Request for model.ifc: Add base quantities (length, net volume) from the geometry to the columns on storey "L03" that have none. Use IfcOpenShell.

First a look at what the model holds.

```python
import ifcopenshell
import ifcopenshell.util.element
import ifcopenshell.util.unit

model = ifcopenshell.open("model.ifc")
print(model.schema)
for unit_type in ("LENGTHUNIT", "AREAUNIT", "VOLUMEUNIT"):
    print(unit_type, ifcopenshell.util.unit.calculate_unit_scale(model, unit_type))
storey = next(s for s in model.by_type("IfcBuildingStorey") if s.Name == "L03")
columns = [e for e in ifcopenshell.util.element.get_decomposition(storey) if e.is_a("IfcColumn")]
for e in sorted(columns, key=lambda e: e.id()):
    print(e.id(), e.is_a(), e.Name, list(ifcopenshell.util.element.get_psets(e, qtos_only=True)), sep=" | ")
```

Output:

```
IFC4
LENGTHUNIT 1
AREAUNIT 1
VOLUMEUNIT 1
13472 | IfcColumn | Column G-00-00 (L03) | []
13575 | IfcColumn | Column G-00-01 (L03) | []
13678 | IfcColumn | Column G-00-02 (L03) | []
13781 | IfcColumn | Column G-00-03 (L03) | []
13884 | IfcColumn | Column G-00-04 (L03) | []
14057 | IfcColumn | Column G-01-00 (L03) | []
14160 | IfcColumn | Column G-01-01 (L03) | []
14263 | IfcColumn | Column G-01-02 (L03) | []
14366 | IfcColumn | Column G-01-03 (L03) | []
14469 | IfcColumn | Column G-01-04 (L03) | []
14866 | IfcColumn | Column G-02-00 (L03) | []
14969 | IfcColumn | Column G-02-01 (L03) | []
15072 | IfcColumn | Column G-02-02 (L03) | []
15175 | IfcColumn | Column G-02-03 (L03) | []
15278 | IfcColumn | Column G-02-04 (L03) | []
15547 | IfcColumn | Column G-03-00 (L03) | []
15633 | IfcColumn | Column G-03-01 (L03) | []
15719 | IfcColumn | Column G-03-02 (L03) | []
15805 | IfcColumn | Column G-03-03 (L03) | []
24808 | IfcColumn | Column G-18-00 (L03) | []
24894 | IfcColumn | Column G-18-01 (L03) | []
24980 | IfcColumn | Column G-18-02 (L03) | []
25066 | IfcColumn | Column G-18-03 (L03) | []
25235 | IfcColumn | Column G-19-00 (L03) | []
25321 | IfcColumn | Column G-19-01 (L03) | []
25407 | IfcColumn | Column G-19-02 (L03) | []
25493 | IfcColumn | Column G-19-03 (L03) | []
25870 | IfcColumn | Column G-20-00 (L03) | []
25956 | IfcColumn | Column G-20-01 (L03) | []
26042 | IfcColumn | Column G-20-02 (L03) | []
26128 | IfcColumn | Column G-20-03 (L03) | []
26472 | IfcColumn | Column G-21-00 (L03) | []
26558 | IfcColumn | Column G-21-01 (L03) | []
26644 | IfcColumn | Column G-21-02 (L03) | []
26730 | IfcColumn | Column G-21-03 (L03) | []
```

```python
import ifcopenshell
import ifcopenshell.api.pset
import ifcopenshell.geom
import ifcopenshell.util.element
import ifcopenshell.util.shape
import ifcopenshell.util.unit

model = ifcopenshell.open("model.ifc")
unit_scale = ifcopenshell.util.unit.calculate_unit_scale(model)
volume_scale = ifcopenshell.util.unit.calculate_unit_scale(model, "VOLUMEUNIT")
settings = ifcopenshell.geom.settings()

storey = next(s for s in model.by_type("IfcBuildingStorey") if s.Name == "L03")
columns = [e for e in ifcopenshell.util.element.get_decomposition(storey) if e.is_a("IfcColumn")]

for e in sorted(columns, key=lambda e: e.id()):
    if ifcopenshell.util.element.get_psets(e, qtos_only=True, should_inherit=False):
        continue
    # Geometry comes back in metres, in the element's own axes.
    shape = ifcopenshell.geom.create_shape(settings, e)
    values = {
        "Length": ifcopenshell.util.shape.get_z(shape.geometry) / unit_scale,
        "NetVolume": ifcopenshell.util.shape.get_volume(shape.geometry) / volume_scale,
    }
    qto = ifcopenshell.api.pset.add_qto(model, product=e, name="Qto_ColumnBaseQuantities")
    ifcopenshell.api.pset.edit_qto(model, qto=qto, properties=values)
    print(e.id(), {k: round(v, 3) for k, v in values.items()})

model.write("model-out.ifc")
```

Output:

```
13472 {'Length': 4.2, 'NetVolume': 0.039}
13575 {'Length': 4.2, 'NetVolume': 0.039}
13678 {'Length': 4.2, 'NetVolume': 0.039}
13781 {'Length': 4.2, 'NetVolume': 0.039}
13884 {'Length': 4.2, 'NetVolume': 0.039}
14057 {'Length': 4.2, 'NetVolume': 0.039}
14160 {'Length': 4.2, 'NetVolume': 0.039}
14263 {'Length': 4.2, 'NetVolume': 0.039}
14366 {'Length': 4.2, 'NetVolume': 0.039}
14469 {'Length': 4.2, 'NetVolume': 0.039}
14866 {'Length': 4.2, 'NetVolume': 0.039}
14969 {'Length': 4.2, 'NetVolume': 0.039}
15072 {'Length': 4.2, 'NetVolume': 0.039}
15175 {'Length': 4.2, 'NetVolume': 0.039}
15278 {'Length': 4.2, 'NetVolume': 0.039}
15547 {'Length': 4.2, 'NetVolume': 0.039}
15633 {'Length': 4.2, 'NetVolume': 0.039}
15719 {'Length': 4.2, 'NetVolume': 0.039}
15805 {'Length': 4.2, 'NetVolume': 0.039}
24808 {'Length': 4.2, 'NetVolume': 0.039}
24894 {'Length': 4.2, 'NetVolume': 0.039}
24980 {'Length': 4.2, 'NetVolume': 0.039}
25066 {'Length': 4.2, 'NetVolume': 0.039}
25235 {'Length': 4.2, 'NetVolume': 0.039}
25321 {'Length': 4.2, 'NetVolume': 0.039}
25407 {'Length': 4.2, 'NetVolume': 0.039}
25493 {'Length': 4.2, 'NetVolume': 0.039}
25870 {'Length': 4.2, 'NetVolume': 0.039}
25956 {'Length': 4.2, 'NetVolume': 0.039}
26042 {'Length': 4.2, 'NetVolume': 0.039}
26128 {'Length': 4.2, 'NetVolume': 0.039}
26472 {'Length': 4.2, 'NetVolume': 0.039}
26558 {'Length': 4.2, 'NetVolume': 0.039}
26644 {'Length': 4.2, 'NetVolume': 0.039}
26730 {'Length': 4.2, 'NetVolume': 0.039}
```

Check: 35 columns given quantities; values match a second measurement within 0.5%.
